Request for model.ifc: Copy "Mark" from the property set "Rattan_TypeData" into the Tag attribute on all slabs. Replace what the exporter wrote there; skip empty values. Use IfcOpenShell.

First a look at what the model holds.

```python
import ifcopenshell
import ifcopenshell.util.element

model = ifcopenshell.open("model.ifc")
print(model.schema)
slabs = model.by_type("IfcSlab")
print(len(slabs), "slabs")
for e in slabs[:8]:
    source = ifcopenshell.util.element.get_pset(e, "Rattan_TypeData", "Mark")
    target = e.Tag
    print(e.id(), repr(source), repr(target), sep=" | ")
```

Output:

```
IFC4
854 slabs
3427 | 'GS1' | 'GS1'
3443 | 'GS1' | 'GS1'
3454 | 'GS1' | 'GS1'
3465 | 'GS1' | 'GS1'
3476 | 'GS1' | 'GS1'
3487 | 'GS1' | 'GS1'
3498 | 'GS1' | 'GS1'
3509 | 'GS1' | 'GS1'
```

```python
import ifcopenshell
import ifcopenshell.util.element

model = ifcopenshell.open("model.ifc")

count = 0
for e in model.by_type("IfcSlab"):
    value = ifcopenshell.util.element.get_pset(e, "Rattan_TypeData", "Mark")
    current = e.Tag
    if not value or not value.strip() or current == value:
        continue
    e.Tag = value
    count += 1

print(count, "slabs updated")

model.write("model_edited.ifc")
```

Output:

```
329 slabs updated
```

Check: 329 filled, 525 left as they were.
